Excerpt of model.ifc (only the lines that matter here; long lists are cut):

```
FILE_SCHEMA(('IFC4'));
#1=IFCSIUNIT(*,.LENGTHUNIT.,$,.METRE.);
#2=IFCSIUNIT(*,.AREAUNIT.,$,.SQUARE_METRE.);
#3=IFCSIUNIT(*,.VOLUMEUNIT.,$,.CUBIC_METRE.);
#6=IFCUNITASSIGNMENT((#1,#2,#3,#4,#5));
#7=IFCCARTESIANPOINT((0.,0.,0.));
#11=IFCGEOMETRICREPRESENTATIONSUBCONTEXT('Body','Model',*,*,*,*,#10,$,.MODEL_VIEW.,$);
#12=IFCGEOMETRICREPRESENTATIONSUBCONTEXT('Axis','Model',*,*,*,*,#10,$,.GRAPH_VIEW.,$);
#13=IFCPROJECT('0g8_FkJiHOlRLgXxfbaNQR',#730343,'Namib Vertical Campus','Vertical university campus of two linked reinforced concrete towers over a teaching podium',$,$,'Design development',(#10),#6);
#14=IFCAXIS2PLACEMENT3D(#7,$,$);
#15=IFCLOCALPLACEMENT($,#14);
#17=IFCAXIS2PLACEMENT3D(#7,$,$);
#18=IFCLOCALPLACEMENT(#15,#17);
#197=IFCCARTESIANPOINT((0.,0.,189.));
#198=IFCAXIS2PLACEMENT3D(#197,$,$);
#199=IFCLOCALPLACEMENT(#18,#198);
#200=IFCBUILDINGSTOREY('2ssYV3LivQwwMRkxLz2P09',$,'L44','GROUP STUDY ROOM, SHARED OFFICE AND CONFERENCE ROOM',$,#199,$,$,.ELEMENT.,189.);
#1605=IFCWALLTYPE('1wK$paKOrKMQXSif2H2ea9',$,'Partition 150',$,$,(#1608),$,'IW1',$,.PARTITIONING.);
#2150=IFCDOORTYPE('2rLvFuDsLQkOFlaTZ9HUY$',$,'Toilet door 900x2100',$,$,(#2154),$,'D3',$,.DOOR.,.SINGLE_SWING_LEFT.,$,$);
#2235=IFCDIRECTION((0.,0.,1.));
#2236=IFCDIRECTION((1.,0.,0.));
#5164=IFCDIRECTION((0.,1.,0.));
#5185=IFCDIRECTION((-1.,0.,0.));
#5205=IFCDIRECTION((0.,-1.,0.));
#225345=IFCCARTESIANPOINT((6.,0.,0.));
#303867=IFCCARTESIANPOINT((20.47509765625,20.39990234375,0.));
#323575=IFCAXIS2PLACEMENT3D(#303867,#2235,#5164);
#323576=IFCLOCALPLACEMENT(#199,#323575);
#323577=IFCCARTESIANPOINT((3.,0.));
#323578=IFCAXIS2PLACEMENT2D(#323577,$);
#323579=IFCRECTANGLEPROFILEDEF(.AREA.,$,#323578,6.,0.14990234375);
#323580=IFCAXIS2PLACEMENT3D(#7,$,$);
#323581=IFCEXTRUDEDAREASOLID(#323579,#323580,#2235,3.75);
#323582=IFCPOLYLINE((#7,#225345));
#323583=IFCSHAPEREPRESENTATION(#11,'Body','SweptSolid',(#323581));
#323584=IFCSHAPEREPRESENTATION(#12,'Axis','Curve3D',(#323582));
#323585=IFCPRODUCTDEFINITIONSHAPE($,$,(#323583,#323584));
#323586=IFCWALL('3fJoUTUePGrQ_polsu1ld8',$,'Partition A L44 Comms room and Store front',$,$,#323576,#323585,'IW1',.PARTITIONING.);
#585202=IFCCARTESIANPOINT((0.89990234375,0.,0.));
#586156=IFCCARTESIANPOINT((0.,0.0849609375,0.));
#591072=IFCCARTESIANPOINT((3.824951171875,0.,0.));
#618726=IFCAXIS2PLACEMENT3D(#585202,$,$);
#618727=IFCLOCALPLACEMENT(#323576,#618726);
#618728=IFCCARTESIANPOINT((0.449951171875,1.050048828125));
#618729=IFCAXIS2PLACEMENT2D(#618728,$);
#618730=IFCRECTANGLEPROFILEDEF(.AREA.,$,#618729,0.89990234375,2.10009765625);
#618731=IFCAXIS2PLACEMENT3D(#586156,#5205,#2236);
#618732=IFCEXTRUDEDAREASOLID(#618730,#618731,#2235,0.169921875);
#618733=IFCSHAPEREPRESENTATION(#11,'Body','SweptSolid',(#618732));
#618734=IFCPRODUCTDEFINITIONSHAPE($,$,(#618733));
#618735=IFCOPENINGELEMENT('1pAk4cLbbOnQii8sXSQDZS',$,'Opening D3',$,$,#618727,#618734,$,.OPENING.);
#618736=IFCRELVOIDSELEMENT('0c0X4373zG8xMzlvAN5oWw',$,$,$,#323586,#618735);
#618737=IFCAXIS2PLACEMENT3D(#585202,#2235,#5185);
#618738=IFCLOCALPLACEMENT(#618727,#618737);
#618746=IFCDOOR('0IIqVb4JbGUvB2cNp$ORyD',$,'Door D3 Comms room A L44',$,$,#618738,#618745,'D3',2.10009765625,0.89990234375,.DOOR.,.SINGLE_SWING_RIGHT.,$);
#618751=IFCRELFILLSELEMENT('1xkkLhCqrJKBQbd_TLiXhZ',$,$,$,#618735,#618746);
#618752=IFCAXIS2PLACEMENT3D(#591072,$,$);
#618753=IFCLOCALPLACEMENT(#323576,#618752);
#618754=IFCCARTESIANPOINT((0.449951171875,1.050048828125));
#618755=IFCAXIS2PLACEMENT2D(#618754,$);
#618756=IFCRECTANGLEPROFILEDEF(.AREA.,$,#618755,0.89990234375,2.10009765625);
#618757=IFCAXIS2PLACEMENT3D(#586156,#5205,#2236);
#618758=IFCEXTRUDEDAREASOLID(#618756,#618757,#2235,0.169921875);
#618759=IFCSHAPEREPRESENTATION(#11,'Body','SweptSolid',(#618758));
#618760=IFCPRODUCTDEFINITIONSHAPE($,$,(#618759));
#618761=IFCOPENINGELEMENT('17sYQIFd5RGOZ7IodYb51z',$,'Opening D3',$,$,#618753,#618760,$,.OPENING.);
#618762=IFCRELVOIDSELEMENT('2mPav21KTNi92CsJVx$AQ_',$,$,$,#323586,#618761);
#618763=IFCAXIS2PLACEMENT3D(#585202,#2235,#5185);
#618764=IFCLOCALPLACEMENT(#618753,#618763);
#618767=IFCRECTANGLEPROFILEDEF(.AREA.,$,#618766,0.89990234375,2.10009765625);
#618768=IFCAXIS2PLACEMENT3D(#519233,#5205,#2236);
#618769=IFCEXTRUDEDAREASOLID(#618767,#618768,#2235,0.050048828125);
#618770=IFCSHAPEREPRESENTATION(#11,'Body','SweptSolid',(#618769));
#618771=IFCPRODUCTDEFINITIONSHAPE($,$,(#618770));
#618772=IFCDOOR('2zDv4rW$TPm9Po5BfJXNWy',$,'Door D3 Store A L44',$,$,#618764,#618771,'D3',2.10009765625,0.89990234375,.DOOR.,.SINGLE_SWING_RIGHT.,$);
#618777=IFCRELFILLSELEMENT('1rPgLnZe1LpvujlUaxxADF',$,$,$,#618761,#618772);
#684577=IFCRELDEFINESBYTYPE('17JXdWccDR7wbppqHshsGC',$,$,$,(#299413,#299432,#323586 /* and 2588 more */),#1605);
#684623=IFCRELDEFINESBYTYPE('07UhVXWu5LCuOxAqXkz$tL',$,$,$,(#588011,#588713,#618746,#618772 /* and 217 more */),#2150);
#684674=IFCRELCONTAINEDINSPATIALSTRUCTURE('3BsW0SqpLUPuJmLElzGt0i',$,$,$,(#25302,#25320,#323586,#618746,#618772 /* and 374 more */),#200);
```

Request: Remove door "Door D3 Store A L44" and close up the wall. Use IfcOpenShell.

```python
import ifcopenshell
import ifcopenshell.api.feature
import ifcopenshell.api.root
import ifcopenshell.geom
import ifcopenshell.util.shape

model = ifcopenshell.open("model.ifc")
settings = ifcopenshell.geom.settings()


def volume(element):
    """Net volume in cubic metres, openings subtracted."""
    shape = ifcopenshell.geom.create_shape(settings, element)
    return ifcopenshell.util.shape.get_volume(shape.geometry)


door = model.by_guid("2zDv4rW$TPm9Po5BfJXNWy")
opening = door.FillsVoids[0].RelatingOpeningElement
wall = opening.VoidsElements[0].RelatingBuildingElement
before = volume(wall)

ifcopenshell.api.root.remove_product(model, product=door)
ifcopenshell.api.feature.remove_feature(model, feature=opening)

after = volume(wall)

print(f"wall volume {before:.3f} -> {after:.3f} m3")

model.write("model_v2.ifc")
```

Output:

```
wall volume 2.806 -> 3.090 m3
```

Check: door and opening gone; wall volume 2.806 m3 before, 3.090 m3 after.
